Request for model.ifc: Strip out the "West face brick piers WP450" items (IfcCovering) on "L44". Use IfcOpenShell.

First a look at what the model holds.

```python
import ifcopenshell
import ifcopenshell.util.element

model = ifcopenshell.open("model.ifc")
print(model.schema)
storey = next(s for s in model.by_type("IfcBuildingStorey") if s.Name == "L44")
coverings = [e for e in ifcopenshell.util.element.get_decomposition(storey) if e.is_a("IfcCovering")]
seen = {}
for e in coverings:
    element_type = ifcopenshell.util.element.get_type(e)
    name = element_type.Name if element_type not in (None, e) else None
    seen[name] = seen.get(name, 0) + 1
for name, count in sorted(seen.items(), key=str):
    print(count, "x", name)
```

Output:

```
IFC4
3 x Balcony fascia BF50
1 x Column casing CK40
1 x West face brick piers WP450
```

```python
import ifcopenshell
import ifcopenshell.api.root
import ifcopenshell.util.element

model = ifcopenshell.open("model.ifc")

storey = next(s for s in model.by_type("IfcBuildingStorey") if s.Name == "L44")
coverings = [e for e in ifcopenshell.util.element.get_decomposition(storey) if e.is_a("IfcCovering")]
targets = [e for e in coverings if (t := ifcopenshell.util.element.get_type(e)) not in (None, e) and t.Name == "West face brick piers WP450"]

for e in targets:
    ifcopenshell.api.root.remove_product(model, product=e)
print(len(targets), "removed")

model.write("model_updated.ifc")
```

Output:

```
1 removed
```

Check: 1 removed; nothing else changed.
